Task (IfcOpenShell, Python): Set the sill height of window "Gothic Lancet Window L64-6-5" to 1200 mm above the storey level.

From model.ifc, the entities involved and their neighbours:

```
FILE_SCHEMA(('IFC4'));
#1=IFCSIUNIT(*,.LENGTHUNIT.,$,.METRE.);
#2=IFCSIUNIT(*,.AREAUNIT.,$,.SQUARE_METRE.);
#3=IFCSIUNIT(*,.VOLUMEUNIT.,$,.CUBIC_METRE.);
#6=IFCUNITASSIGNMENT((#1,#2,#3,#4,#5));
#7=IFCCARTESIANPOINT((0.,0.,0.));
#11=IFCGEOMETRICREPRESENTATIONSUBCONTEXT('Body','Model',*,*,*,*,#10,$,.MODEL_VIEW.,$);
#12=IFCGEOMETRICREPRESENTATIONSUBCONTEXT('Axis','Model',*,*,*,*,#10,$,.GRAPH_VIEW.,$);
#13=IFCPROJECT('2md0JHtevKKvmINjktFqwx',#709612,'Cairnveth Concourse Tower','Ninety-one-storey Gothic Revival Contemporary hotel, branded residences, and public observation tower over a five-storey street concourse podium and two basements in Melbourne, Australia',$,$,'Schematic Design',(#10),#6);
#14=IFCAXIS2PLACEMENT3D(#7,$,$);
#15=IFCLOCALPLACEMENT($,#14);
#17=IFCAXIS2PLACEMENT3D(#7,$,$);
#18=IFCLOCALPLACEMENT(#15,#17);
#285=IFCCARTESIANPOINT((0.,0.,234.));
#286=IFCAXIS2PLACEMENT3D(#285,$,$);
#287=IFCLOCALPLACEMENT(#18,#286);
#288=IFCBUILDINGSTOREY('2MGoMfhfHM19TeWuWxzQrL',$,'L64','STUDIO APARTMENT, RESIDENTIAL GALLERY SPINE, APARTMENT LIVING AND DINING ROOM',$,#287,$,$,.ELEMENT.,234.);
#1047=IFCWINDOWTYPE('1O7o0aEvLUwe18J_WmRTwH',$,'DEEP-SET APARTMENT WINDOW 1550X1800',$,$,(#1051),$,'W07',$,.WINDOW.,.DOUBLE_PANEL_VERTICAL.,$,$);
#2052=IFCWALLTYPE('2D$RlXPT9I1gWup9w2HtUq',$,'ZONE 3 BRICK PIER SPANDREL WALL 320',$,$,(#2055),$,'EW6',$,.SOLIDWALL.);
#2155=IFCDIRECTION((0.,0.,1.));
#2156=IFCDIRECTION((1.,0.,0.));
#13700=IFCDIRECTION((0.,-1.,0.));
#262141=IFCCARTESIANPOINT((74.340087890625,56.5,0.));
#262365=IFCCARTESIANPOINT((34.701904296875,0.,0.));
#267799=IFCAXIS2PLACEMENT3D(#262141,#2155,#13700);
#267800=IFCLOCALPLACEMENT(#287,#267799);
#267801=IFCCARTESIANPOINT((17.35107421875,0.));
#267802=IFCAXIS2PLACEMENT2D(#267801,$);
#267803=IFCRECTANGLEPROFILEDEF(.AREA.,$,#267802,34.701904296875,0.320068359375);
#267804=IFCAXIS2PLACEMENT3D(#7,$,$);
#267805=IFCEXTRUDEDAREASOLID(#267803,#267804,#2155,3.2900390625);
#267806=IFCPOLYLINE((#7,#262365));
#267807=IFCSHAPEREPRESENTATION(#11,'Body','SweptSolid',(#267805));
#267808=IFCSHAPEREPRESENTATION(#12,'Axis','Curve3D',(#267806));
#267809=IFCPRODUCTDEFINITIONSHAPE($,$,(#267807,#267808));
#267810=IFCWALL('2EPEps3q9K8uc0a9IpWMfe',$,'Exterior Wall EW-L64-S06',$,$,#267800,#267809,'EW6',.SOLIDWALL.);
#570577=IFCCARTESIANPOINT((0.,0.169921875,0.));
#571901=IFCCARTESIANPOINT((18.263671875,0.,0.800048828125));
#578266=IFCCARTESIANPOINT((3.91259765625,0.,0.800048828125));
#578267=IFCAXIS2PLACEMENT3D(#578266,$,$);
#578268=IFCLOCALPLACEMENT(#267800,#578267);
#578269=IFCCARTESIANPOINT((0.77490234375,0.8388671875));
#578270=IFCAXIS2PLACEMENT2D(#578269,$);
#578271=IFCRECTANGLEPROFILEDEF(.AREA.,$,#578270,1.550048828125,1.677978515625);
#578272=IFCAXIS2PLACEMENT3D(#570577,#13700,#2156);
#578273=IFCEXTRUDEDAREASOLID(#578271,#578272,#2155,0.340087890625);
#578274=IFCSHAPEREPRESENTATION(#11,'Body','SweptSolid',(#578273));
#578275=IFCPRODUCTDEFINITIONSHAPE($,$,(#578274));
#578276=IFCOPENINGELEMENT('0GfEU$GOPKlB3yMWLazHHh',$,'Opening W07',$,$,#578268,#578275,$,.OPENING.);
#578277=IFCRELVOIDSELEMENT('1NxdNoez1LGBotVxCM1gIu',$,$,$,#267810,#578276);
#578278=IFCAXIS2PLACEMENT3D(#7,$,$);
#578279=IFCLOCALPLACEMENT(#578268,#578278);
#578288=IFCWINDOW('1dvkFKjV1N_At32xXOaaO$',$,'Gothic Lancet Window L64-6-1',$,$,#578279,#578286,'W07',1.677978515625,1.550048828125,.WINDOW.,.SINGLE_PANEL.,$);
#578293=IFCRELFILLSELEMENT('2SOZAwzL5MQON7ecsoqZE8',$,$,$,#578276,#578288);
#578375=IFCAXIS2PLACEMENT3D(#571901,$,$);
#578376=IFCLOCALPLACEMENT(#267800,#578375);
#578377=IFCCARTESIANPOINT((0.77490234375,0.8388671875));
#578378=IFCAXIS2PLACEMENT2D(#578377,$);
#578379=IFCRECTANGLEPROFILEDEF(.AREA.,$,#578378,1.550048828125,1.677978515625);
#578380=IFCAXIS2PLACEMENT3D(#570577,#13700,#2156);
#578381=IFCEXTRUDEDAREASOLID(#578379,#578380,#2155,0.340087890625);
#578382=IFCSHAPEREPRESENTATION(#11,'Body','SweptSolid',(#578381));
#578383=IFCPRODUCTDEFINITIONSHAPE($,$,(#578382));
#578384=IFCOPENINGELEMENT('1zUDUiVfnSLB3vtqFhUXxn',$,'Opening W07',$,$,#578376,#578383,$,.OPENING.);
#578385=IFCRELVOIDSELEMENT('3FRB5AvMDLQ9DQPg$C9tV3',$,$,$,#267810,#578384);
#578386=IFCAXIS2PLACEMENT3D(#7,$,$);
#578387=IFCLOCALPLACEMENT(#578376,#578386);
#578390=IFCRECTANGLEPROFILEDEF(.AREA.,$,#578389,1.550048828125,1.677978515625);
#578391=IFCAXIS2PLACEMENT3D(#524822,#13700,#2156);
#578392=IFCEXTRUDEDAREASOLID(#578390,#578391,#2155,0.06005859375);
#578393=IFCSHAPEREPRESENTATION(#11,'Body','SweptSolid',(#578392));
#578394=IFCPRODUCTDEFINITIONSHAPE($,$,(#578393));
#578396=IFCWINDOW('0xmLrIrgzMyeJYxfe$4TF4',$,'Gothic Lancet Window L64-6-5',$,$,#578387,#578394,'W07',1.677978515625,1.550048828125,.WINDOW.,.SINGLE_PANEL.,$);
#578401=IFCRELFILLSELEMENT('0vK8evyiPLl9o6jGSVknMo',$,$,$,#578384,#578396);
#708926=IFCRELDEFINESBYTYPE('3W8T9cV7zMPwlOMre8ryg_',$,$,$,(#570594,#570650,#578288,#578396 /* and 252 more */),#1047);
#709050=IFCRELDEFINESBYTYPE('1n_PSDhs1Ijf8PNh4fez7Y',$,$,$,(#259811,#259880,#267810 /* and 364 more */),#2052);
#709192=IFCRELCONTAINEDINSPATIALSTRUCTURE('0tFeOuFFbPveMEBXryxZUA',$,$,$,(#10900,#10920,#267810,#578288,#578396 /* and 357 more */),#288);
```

```python
import numpy as np
import ifcopenshell
import ifcopenshell.api.geometry
import ifcopenshell.geom
import ifcopenshell.util.element
import ifcopenshell.util.placement
import ifcopenshell.util.shape
import ifcopenshell.util.unit

model = ifcopenshell.open("model.ifc")
unit_scale = ifcopenshell.util.unit.calculate_unit_scale(model)

window = model.by_guid("0xmLrIrgzMyeJYxfe$4TF4")
opening = window.FillsVoids[0].RelatingOpeningElement
storey = ifcopenshell.util.element.get_container(window, ifc_class="IfcBuildingStorey")
level = ifcopenshell.util.placement.get_local_placement(storey.ObjectPlacement)[2, 3]

# The opening's origin need not be at the sill, so measure its lowest point.
shape = ifcopenshell.geom.create_shape(ifcopenshell.geom.settings(), opening)
bottom = ifcopenshell.util.shape.get_shape_bottom_elevation(shape, shape.geometry) / unit_scale
dz = level + 1.2 / unit_scale - bottom

shift = np.array([0.0, 0.0, dz])
# The window is placed relative to its opening, so it follows when the opening moves.
matrix = ifcopenshell.util.placement.get_local_placement(opening.ObjectPlacement)
matrix[:3, 3] += shift
ifcopenshell.api.geometry.edit_object_placement(
    model, product=opening, matrix=matrix, is_si=False, should_transform_children=True
)

print(f"moved by {dz * unit_scale:+.3f} m")

model.write("model_edited.ifc")
```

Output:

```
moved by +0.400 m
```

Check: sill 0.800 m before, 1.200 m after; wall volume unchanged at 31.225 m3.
